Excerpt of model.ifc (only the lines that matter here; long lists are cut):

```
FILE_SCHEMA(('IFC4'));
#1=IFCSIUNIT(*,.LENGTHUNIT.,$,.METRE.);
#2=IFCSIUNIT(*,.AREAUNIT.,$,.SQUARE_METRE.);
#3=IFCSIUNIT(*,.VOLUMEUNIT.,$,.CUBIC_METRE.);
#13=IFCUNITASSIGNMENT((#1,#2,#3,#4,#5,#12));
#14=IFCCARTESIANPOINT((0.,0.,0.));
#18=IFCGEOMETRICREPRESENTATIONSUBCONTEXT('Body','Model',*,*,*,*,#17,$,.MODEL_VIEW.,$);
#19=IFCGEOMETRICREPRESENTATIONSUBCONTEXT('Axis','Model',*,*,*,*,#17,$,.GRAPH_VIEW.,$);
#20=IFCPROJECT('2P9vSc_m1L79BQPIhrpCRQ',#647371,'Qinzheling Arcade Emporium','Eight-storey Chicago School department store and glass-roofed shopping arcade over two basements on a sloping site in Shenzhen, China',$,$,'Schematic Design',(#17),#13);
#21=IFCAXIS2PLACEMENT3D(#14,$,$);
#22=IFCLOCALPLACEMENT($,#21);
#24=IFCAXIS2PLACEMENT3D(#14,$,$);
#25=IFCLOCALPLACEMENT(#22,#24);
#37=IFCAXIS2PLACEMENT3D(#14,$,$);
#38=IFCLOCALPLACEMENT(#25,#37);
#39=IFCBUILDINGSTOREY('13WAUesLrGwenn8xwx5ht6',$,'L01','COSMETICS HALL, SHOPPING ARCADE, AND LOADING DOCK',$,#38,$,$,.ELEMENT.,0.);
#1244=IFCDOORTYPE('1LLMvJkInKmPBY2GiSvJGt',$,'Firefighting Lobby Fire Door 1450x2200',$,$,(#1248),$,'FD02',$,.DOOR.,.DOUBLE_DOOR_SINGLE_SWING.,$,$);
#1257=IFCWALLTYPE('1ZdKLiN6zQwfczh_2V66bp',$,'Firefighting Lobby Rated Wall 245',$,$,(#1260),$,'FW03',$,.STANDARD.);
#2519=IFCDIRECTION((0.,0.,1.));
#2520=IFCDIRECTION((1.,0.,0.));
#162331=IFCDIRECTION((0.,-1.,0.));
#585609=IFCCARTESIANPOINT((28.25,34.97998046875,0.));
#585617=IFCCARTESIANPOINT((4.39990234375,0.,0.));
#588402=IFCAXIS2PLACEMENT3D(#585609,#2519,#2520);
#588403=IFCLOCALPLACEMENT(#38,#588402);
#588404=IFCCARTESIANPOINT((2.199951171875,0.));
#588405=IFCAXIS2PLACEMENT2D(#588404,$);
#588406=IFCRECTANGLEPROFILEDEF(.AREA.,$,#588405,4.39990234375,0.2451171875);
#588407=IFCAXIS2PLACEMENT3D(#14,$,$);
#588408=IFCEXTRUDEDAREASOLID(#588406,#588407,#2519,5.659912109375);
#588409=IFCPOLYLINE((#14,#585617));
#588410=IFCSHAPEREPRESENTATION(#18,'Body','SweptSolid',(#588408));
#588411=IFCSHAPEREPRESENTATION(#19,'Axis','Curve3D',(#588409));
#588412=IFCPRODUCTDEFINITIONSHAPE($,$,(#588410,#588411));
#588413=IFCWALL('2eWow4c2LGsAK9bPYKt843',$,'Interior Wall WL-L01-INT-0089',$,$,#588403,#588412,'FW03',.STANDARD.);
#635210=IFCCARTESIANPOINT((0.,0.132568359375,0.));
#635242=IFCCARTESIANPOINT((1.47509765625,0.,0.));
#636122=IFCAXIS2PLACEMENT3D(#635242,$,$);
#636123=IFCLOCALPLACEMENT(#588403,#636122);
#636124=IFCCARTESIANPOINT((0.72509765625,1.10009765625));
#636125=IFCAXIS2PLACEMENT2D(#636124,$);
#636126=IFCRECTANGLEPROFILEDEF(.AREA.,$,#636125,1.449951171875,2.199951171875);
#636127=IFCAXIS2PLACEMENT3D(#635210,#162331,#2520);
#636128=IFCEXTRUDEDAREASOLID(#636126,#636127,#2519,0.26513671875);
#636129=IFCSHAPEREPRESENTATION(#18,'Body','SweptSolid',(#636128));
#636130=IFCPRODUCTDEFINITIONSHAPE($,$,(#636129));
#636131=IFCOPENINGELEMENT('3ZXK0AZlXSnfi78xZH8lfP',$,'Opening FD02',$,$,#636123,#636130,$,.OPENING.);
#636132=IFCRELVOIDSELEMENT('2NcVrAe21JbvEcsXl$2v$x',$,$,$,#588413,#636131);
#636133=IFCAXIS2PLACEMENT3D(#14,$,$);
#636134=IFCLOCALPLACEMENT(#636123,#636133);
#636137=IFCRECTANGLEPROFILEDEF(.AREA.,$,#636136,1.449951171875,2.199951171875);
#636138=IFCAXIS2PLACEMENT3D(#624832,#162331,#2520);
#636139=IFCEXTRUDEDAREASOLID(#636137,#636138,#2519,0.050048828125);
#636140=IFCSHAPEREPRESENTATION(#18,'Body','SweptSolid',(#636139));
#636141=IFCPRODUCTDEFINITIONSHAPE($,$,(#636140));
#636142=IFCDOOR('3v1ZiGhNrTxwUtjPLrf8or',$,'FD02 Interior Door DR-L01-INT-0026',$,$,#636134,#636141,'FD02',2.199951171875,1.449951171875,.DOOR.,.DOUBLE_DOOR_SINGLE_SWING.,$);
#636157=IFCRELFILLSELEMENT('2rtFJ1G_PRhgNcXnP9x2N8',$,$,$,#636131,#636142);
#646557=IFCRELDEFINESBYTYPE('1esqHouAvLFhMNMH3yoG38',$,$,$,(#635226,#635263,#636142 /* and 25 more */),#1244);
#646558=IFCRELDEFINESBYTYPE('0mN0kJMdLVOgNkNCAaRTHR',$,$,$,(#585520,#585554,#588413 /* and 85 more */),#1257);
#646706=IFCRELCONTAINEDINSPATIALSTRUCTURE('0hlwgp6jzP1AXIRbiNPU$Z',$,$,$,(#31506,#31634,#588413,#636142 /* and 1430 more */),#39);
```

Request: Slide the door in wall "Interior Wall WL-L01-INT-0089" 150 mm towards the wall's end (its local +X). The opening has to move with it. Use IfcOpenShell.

```python
import ifcopenshell
import ifcopenshell.api.geometry
import ifcopenshell.util.placement

model = ifcopenshell.open("model.ifc")

door = model.by_id(636142)
opening = door.FillsVoids[0].RelatingOpeningElement
wall = opening.VoidsElements[0].RelatingBuildingElement

wall_matrix = ifcopenshell.util.placement.get_local_placement(wall.ObjectPlacement)
shift = wall_matrix[:3, 0] * 0.15
before = ifcopenshell.util.placement.get_local_placement(door.ObjectPlacement)[:3, 3].copy()

# The door is placed relative to its opening, so it follows when the opening moves.
matrix = ifcopenshell.util.placement.get_local_placement(opening.ObjectPlacement)
matrix[:3, 3] += shift
ifcopenshell.api.geometry.edit_object_placement(
    model, product=opening, matrix=matrix, is_si=False, should_transform_children=True
)

after = ifcopenshell.util.placement.get_local_placement(door.ObjectPlacement)[:3, 3]
print("door moved by", (after - before).round(3) + 0.0)

model.write("model_rev.ifc")
```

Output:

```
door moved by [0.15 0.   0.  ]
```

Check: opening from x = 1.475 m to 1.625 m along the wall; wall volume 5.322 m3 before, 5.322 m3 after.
